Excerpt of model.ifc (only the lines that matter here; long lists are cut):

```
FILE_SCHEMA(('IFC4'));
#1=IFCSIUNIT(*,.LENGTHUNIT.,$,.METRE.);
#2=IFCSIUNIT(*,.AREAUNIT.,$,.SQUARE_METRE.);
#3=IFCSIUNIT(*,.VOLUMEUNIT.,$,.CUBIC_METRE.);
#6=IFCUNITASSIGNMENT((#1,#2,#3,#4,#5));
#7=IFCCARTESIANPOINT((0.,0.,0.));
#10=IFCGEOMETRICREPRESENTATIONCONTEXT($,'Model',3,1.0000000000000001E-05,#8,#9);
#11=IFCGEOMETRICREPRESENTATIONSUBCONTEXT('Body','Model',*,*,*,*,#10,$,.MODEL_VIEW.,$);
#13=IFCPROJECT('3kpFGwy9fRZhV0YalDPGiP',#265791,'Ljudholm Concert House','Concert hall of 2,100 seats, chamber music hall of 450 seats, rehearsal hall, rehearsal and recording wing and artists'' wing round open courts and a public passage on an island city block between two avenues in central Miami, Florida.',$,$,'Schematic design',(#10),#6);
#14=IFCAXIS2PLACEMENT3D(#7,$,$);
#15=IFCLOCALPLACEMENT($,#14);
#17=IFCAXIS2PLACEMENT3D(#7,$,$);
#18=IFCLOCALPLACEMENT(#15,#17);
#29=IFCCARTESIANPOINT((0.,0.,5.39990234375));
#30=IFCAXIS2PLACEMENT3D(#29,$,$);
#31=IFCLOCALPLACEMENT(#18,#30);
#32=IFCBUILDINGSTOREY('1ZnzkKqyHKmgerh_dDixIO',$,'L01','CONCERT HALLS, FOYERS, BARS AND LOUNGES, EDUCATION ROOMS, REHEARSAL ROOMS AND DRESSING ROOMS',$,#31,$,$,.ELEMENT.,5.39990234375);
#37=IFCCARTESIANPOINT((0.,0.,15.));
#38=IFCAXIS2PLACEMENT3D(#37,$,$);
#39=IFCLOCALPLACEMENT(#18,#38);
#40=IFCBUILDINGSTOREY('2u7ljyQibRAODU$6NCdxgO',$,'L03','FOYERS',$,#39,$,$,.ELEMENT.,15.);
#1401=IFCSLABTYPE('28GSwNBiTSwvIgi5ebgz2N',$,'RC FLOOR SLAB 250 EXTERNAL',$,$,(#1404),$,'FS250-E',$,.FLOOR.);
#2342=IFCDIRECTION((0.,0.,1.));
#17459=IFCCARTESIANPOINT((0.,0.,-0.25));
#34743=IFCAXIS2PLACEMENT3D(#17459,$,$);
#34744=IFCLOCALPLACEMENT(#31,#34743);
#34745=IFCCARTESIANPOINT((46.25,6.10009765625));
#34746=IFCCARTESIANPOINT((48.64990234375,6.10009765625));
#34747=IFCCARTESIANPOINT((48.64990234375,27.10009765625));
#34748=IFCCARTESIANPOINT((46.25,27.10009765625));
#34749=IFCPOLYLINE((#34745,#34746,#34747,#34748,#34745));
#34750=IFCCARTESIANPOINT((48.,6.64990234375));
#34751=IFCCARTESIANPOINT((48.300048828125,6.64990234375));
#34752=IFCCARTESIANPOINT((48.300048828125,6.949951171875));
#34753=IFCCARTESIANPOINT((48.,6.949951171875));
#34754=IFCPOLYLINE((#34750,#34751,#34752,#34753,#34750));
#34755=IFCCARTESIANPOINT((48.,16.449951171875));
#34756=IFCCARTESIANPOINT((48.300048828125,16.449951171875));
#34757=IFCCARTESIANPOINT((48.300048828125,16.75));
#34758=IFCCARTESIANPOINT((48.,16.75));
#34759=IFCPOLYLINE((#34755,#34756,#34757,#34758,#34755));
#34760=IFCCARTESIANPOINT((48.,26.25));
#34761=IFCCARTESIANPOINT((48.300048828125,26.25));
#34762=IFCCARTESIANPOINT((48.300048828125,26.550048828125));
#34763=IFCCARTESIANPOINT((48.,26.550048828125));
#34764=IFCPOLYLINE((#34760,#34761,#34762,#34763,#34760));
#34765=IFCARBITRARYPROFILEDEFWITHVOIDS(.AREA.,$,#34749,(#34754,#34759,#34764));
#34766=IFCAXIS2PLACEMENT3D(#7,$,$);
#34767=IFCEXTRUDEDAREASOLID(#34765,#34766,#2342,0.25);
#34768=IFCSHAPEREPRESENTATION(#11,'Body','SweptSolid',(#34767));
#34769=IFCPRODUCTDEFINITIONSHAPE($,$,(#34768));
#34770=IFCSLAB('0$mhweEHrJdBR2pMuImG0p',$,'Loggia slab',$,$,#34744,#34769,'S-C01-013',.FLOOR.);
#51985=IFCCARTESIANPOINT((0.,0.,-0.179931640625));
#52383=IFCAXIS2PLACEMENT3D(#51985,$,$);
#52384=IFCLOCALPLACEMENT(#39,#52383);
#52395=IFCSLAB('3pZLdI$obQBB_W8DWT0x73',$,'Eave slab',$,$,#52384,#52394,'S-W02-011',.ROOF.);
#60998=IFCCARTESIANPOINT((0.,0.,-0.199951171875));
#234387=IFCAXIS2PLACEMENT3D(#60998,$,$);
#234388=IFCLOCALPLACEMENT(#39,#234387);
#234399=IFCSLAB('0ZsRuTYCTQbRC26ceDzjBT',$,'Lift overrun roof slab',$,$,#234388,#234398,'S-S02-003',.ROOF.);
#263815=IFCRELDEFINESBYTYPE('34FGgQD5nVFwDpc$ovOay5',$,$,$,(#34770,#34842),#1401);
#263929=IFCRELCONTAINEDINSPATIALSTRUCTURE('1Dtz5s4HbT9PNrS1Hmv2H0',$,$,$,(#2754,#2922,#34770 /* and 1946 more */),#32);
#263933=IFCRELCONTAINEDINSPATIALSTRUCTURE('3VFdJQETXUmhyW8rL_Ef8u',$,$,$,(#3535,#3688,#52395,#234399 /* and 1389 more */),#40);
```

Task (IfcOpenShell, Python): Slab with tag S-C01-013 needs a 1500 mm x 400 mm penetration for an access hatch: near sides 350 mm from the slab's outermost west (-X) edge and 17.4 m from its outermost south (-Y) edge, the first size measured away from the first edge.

```python
import numpy as np
import ifcopenshell
import ifcopenshell.api.feature
import ifcopenshell.api.geometry
import ifcopenshell.api.root
import ifcopenshell.geom
import ifcopenshell.util.placement
import ifcopenshell.util.representation
import ifcopenshell.util.shape
import ifcopenshell.util.unit

model = ifcopenshell.open("model.ifc")
unit_scale = ifcopenshell.util.unit.calculate_unit_scale(model)
settings = ifcopenshell.geom.settings()


def volume(element):
    """Net volume in cubic metres, openings subtracted."""
    shape = ifcopenshell.geom.create_shape(settings, element)
    return ifcopenshell.util.shape.get_volume(shape.geometry)


slab = model.by_guid("0$mhweEHrJdBR2pMuImG0p")
before = volume(slab)

# Extent in the slab's own axes, in metres. The edges named are its -X and -Y sides.
slab_shape = ifcopenshell.geom.create_shape(settings, slab)
vertices = ifcopenshell.util.shape.get_vertices(slab_shape.geometry)
x_min, y_min, bottom = vertices.min(axis=0)
top = vertices[:, 2].max()

opening = ifcopenshell.api.root.create_entity(model, ifc_class="IfcOpeningElement", name="Access hatch opening", predefined_type="OPENING")
context = ifcopenshell.util.representation.get_context(model, "Model", "Body", "MODEL_VIEW")
width, depth = 1.5, 0.4
outline = [(0.0, 0.0), (width, 0.0), (width, depth), (0.0, depth), (0.0, 0.0)]
# Overshoot both faces by 50 mm so the cut is clean.
shape = ifcopenshell.api.geometry.add_slab_representation(
    model, context=context, depth=top - bottom + 0.1, polyline=outline
)
ifcopenshell.api.geometry.assign_representation(model, product=opening, representation=shape)

matrix = ifcopenshell.util.placement.get_local_placement(slab.ObjectPlacement)
matrix[:, 3] = matrix @ np.append(np.array([x_min + 0.35, y_min + 17.4, bottom - 0.05]) / unit_scale, 1.0)
ifcopenshell.api.geometry.edit_object_placement(model, product=opening, matrix=matrix, is_si=False)
ifcopenshell.api.feature.add_feature(model, feature=opening, element=slab)

after = volume(slab)

print(f"slab volume {before:.3f} -> {after:.3f} m3")

model.write("model-out.ifc")
```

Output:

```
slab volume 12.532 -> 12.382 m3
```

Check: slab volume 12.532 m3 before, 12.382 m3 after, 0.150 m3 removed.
